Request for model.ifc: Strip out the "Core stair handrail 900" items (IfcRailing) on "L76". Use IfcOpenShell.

First a look at what the model holds.

```python
import ifcopenshell
import ifcopenshell.util.element

model = ifcopenshell.open("model.ifc")
print(model.schema)
storey = next(s for s in model.by_type("IfcBuildingStorey") if s.Name == "L76")
railings = [e for e in ifcopenshell.util.element.get_decomposition(storey) if e.is_a("IfcRailing")]
seen = {}
for e in railings:
    element_type = ifcopenshell.util.element.get_type(e)
    name = element_type.Name if element_type not in (None, e) else None
    seen[name] = seen.get(name, 0) + 1
for name, count in sorted(seen.items(), key=str):
    print(count, "x", name)
```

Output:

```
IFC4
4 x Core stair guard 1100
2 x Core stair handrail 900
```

```python
import ifcopenshell
import ifcopenshell.api.root
import ifcopenshell.util.element

model = ifcopenshell.open("model.ifc")

storey = next(s for s in model.by_type("IfcBuildingStorey") if s.Name == "L76")
railings = [e for e in ifcopenshell.util.element.get_decomposition(storey) if e.is_a("IfcRailing")]
targets = [e for e in railings if (t := ifcopenshell.util.element.get_type(e)) not in (None, e) and t.Name == "Core stair handrail 900"]

for e in targets:
    ifcopenshell.api.root.remove_product(model, product=e)
print(len(targets), "removed")

model.write("model_updated.ifc")
```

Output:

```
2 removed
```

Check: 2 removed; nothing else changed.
